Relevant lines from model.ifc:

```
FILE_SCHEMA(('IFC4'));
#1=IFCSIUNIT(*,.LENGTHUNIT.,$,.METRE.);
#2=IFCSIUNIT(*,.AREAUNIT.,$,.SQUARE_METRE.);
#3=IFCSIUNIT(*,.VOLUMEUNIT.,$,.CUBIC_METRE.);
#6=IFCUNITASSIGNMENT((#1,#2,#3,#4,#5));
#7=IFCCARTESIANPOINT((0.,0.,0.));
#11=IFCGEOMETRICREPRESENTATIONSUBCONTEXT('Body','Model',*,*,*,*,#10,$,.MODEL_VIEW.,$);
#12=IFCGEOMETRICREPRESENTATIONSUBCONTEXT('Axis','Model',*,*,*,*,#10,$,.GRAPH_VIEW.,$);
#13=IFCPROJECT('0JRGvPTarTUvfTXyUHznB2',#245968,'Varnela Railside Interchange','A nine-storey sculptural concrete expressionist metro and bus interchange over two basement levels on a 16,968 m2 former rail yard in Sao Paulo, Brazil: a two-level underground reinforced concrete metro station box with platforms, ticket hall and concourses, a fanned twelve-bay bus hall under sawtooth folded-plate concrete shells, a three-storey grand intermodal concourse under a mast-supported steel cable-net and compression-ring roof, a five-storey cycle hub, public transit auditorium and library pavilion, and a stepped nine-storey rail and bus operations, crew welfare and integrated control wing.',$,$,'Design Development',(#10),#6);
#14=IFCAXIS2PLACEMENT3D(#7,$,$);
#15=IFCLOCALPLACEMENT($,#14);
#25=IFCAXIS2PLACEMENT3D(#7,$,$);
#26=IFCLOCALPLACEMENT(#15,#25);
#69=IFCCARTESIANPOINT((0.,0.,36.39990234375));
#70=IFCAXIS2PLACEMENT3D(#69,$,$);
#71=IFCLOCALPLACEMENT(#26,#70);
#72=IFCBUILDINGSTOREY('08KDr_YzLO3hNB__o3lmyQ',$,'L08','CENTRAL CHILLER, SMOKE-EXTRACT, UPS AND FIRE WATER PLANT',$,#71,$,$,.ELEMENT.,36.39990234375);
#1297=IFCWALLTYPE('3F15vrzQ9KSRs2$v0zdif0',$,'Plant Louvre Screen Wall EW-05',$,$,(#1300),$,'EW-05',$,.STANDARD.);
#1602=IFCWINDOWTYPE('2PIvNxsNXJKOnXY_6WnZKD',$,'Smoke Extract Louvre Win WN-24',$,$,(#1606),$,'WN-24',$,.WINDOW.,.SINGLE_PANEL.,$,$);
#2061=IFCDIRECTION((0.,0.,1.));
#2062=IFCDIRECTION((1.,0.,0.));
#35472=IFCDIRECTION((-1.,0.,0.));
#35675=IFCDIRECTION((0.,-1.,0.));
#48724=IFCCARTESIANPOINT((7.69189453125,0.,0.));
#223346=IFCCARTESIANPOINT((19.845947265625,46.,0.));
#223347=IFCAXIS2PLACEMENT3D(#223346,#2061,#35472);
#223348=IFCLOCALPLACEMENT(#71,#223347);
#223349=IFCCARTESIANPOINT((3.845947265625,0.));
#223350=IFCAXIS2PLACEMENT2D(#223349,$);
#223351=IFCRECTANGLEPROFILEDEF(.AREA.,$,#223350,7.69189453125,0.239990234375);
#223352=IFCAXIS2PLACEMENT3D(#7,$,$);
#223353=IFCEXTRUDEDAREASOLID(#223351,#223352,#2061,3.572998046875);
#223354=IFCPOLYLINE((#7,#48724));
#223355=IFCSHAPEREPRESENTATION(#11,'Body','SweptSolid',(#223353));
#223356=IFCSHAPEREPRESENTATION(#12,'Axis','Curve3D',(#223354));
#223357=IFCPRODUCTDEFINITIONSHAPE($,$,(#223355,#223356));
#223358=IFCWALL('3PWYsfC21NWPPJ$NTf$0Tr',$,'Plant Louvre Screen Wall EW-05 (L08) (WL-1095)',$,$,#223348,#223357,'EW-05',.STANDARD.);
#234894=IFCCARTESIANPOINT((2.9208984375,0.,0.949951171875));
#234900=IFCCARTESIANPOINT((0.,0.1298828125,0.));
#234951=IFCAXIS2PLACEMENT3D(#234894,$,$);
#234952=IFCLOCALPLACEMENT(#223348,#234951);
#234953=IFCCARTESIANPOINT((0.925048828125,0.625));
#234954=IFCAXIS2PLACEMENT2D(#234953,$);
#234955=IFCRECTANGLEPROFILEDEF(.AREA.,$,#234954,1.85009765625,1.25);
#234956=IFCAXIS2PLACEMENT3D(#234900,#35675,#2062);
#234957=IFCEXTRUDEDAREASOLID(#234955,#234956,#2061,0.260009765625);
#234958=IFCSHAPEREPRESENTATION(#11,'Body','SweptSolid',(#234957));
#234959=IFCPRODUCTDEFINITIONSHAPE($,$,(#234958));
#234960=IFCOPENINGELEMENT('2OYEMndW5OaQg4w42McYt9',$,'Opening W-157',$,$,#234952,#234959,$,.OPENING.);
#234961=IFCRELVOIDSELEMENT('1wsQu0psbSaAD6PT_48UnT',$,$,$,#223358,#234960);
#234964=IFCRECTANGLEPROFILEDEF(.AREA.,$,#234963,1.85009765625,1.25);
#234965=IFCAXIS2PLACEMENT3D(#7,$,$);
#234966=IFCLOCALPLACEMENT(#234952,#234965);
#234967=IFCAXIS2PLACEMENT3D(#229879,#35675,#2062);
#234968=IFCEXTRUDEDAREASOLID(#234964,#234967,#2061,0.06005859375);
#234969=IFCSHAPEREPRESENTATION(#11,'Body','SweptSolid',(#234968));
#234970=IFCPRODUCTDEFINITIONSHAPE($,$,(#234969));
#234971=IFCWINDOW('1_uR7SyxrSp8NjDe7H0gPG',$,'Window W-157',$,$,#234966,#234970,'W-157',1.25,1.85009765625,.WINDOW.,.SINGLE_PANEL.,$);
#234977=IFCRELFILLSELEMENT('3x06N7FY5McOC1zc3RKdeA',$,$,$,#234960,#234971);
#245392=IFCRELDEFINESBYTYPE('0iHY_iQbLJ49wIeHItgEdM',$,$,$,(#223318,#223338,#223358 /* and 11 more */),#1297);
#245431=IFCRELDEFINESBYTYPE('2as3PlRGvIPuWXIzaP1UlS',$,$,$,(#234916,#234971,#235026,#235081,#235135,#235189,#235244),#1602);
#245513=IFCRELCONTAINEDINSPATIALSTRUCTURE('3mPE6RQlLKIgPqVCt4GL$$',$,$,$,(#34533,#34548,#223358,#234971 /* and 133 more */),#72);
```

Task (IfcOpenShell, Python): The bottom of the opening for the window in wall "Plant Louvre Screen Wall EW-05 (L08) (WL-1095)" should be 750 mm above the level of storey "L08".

```python
import numpy as np
import ifcopenshell
import ifcopenshell.api.geometry
import ifcopenshell.geom
import ifcopenshell.util.element
import ifcopenshell.util.placement
import ifcopenshell.util.shape
import ifcopenshell.util.unit

model = ifcopenshell.open("model.ifc")
unit_scale = ifcopenshell.util.unit.calculate_unit_scale(model)

window = model.by_guid("1_uR7SyxrSp8NjDe7H0gPG")
opening = window.FillsVoids[0].RelatingOpeningElement
storey = ifcopenshell.util.element.get_container(window, ifc_class="IfcBuildingStorey")
level = ifcopenshell.util.placement.get_local_placement(storey.ObjectPlacement)[2, 3]

# The opening's origin need not be at the sill, so measure its lowest point.
shape = ifcopenshell.geom.create_shape(ifcopenshell.geom.settings(), opening)
bottom = ifcopenshell.util.shape.get_shape_bottom_elevation(shape, shape.geometry) / unit_scale
dz = level + 0.75 - bottom

shift = np.array([0.0, 0.0, dz])
# The window is placed relative to its opening, so it follows when the opening moves.
matrix = ifcopenshell.util.placement.get_local_placement(opening.ObjectPlacement)
matrix[:3, 3] += shift
ifcopenshell.api.geometry.edit_object_placement(
    model, product=opening, matrix=matrix, is_si=False, should_transform_children=True
)

print(f"moved by {dz * unit_scale:+.3f} m")

model.write("model_v2.ifc")
```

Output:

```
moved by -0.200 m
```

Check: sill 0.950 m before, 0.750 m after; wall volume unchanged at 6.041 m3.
